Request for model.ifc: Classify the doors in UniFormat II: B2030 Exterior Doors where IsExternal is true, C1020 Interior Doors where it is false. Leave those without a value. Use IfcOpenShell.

First a look at what the model holds.

```python
import ifcopenshell
import ifcopenshell.util.element

model = ifcopenshell.open("model.ifc")
print(model.schema)
print("classifications:", [c.Name for c in model.by_type("IfcClassification")])
values = [ifcopenshell.util.element.get_pset(e, "Pset_DoorCommon", "IsExternal") for e in model.by_type("IfcDoor")]
for value in (True, False, None):
    print("IsExternal", value, values.count(value))
```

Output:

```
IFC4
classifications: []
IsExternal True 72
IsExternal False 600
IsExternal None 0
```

```python
import ifcopenshell
import ifcopenshell.api.classification
import ifcopenshell.util.element

model = ifcopenshell.open("model.ifc")

system = ifcopenshell.api.classification.add_classification(model, classification="UniFormat II")

doors = model.by_type("IfcDoor")
external = {e: ifcopenshell.util.element.get_pset(e, "Pset_DoorCommon", "IsExternal") for e in doors}
for flag, code, name in ((True, "B2030", "Exterior Doors"), (False, "C1020", "Interior Doors")):
    products = [e for e in doors if external[e] is flag]
    ifcopenshell.api.classification.add_reference(
        model, products=products, classification=system, identification=code, name=name
    )
    print(code, len(products))

model.write("model_updated.ifc")
```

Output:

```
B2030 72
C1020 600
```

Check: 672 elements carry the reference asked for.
